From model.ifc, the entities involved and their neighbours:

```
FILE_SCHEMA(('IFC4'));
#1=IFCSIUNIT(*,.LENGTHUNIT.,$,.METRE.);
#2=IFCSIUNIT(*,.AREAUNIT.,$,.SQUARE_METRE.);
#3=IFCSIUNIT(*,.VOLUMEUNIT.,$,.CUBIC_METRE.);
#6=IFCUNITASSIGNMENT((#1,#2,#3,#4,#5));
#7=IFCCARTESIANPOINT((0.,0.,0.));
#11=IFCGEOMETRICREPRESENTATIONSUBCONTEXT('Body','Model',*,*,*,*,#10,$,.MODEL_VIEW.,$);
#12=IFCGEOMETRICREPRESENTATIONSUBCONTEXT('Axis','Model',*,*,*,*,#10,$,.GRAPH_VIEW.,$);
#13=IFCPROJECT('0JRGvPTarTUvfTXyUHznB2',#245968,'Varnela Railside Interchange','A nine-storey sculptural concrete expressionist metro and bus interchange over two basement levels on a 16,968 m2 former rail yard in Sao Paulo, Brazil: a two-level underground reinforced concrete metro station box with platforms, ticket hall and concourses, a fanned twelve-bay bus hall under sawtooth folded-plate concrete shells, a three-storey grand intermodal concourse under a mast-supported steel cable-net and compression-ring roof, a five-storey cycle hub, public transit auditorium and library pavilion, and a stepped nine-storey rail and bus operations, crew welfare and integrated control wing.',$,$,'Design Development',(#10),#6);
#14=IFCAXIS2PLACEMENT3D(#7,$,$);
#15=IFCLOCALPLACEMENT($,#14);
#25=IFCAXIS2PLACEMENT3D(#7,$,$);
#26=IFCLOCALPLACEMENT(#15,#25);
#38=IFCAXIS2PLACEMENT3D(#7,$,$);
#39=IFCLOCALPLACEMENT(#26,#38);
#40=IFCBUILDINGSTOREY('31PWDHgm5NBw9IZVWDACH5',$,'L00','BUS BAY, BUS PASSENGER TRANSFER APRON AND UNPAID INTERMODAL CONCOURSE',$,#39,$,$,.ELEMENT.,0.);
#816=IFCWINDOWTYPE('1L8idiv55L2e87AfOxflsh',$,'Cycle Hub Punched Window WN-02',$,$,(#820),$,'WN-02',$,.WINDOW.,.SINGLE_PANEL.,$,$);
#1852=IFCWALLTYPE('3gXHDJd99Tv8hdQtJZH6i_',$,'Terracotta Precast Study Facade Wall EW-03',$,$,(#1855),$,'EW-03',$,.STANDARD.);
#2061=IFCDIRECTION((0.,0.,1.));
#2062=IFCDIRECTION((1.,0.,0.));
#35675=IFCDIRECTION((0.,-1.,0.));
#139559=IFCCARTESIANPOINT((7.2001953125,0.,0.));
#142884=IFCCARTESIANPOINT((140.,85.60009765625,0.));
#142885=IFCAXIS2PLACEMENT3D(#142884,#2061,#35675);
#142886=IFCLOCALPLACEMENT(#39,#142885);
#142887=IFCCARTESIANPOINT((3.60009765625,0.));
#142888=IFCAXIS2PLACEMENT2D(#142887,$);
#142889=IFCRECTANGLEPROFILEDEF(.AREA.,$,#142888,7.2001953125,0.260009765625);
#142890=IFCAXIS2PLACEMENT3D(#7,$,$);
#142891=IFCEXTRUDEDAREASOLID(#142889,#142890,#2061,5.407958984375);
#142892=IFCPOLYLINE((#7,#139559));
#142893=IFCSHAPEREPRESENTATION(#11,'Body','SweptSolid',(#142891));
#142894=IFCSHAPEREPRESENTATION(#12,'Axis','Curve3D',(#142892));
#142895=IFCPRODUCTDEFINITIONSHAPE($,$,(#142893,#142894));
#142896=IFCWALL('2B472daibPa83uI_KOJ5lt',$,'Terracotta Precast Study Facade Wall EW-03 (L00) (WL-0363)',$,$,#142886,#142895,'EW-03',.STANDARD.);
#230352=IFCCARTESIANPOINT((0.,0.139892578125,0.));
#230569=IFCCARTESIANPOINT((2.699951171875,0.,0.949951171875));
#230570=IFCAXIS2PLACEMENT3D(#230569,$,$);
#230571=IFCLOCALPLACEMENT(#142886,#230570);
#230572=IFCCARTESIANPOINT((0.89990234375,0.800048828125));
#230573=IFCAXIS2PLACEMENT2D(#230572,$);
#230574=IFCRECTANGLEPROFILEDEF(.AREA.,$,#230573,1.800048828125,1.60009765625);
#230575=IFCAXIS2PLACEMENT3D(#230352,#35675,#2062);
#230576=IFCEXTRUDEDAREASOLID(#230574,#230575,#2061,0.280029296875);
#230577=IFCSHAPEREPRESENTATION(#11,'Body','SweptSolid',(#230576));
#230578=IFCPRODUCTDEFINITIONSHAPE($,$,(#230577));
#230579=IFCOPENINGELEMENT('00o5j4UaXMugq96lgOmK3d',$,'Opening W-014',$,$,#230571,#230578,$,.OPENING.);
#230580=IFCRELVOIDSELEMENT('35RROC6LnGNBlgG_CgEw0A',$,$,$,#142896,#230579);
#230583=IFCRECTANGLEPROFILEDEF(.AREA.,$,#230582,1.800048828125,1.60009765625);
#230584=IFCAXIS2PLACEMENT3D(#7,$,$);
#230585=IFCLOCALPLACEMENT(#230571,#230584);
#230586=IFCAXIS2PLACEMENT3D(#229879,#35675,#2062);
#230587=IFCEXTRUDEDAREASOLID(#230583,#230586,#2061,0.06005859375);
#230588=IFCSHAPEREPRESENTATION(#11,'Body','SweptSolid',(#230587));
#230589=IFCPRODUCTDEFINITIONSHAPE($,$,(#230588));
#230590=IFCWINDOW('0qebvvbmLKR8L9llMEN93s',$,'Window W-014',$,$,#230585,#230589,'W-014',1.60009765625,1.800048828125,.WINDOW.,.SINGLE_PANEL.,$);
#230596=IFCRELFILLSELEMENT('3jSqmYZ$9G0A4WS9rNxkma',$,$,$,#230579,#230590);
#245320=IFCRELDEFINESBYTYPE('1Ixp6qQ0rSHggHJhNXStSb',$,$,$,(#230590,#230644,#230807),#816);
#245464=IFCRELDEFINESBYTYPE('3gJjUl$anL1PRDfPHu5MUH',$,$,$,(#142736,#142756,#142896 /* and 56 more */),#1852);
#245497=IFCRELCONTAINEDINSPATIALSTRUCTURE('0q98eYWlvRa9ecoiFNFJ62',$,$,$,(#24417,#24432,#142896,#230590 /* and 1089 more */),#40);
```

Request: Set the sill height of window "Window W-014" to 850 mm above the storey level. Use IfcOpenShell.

```python
import numpy as np
import ifcopenshell
import ifcopenshell.api.geometry
import ifcopenshell.geom
import ifcopenshell.util.element
import ifcopenshell.util.placement
import ifcopenshell.util.shape
import ifcopenshell.util.unit

model = ifcopenshell.open("model.ifc")
unit_scale = ifcopenshell.util.unit.calculate_unit_scale(model)

window = model.by_guid("0qebvvbmLKR8L9llMEN93s")
opening = window.FillsVoids[0].RelatingOpeningElement
storey = ifcopenshell.util.element.get_container(window, ifc_class="IfcBuildingStorey")
level = ifcopenshell.util.placement.get_local_placement(storey.ObjectPlacement)[2, 3]

# The opening's origin need not be at the sill, so measure its lowest point.
shape = ifcopenshell.geom.create_shape(ifcopenshell.geom.settings(), opening)
bottom = ifcopenshell.util.shape.get_shape_bottom_elevation(shape, shape.geometry) / unit_scale
dz = level + 0.85 / unit_scale - bottom

shift = np.array([0.0, 0.0, dz])
# The window is placed relative to its opening, so it follows when the opening moves.
matrix = ifcopenshell.util.placement.get_local_placement(opening.ObjectPlacement)
matrix[:3, 3] += shift
ifcopenshell.api.geometry.edit_object_placement(
    model, product=opening, matrix=matrix, is_si=False, should_transform_children=True
)

print(f"moved by {dz * unit_scale:+.3f} m")

model.write("model_rev.ifc")
```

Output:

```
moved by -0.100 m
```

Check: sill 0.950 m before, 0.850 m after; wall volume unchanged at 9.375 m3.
